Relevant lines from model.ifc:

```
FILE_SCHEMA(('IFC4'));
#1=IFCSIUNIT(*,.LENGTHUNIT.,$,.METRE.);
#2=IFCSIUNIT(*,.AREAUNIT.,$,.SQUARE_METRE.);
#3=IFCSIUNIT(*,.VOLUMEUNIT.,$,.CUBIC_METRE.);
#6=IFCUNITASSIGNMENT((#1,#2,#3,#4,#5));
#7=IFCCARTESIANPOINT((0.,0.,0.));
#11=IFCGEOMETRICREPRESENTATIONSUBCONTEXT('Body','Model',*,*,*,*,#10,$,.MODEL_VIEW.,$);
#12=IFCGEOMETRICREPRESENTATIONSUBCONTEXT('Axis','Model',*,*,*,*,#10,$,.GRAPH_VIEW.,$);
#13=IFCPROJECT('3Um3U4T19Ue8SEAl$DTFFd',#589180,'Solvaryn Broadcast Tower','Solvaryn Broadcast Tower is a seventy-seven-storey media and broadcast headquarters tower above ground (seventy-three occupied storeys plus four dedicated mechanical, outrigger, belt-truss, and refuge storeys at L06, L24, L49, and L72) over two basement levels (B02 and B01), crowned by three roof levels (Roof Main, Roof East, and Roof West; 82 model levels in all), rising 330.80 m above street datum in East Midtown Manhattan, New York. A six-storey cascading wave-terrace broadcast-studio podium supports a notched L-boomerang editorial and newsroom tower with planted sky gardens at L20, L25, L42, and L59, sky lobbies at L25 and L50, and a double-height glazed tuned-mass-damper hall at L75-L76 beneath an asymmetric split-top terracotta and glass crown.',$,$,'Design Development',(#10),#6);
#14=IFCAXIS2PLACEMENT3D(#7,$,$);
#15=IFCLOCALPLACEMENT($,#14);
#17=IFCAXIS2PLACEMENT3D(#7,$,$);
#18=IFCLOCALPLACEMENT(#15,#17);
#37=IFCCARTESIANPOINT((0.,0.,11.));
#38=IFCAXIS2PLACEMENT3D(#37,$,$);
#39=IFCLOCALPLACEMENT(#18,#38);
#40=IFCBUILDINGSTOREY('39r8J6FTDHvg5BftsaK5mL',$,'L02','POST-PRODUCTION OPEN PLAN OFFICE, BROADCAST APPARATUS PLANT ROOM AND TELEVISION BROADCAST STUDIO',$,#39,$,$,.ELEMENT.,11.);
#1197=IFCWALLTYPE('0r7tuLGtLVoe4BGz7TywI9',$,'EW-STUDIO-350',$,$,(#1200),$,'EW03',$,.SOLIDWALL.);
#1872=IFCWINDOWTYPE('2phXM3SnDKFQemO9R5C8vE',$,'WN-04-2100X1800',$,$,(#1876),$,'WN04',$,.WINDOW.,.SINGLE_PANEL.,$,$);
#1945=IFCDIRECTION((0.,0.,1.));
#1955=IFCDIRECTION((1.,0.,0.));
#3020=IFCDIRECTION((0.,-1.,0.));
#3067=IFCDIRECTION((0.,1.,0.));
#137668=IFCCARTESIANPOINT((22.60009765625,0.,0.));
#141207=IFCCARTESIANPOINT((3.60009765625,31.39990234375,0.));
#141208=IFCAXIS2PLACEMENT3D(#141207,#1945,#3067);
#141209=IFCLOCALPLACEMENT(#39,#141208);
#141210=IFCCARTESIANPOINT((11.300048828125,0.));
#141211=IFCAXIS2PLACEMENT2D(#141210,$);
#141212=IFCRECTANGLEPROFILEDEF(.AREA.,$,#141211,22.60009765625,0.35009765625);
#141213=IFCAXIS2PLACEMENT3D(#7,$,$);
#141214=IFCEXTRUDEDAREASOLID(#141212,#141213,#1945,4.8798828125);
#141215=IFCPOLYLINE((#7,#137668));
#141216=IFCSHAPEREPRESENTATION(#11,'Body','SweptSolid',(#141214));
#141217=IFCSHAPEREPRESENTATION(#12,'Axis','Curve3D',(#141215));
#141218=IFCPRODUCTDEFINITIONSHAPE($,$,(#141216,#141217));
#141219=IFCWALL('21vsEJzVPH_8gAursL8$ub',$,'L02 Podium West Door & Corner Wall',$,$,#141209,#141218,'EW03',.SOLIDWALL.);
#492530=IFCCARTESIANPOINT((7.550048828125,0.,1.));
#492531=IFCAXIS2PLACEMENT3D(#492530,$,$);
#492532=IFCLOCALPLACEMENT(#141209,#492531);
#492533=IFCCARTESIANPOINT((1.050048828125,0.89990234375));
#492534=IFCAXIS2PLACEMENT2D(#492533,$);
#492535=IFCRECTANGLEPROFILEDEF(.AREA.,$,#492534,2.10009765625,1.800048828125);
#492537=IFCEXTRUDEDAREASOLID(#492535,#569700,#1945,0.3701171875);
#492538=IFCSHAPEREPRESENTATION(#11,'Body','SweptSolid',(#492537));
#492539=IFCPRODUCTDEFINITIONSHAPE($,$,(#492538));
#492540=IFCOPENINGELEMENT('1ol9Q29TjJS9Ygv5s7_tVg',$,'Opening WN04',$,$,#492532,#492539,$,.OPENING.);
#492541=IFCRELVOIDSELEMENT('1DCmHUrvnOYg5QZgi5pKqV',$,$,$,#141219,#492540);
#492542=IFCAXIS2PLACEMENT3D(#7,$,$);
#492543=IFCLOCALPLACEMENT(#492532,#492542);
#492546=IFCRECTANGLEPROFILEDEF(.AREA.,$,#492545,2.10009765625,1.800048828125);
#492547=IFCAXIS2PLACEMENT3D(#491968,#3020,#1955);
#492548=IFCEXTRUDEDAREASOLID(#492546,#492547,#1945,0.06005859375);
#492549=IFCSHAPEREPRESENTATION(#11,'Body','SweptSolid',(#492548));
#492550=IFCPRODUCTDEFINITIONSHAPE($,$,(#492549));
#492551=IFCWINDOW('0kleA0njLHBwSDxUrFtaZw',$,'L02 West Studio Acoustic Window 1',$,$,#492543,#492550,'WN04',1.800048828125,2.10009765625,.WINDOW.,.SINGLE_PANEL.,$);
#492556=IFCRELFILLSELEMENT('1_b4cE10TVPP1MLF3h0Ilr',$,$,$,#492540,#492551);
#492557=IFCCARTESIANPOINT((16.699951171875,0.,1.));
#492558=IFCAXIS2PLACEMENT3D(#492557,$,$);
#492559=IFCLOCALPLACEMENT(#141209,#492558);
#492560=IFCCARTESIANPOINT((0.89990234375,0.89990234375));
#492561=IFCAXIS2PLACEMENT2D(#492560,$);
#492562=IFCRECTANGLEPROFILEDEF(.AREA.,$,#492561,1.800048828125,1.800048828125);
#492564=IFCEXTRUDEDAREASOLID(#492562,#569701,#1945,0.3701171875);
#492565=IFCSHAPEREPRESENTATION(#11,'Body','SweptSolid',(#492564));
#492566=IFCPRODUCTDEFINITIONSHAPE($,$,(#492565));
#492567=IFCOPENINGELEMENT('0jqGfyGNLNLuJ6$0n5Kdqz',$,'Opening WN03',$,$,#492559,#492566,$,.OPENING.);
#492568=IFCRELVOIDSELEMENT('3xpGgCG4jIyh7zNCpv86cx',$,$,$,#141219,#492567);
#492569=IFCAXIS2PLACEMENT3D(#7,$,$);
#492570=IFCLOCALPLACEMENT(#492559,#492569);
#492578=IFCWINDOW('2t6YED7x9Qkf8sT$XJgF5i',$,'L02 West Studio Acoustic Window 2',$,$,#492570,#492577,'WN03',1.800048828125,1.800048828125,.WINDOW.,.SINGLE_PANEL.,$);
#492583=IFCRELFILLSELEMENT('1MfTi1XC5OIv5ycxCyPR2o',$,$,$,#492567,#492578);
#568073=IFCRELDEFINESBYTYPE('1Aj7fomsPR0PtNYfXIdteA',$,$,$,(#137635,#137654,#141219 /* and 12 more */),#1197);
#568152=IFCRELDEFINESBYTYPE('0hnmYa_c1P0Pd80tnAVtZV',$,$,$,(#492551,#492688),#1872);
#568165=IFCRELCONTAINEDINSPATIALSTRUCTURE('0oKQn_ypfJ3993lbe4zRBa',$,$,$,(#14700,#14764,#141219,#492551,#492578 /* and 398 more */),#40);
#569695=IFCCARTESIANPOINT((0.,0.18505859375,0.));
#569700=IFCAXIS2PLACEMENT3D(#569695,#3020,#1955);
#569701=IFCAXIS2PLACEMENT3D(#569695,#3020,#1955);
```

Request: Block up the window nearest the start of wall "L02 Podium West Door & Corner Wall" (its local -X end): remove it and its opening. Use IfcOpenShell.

```python
import ifcopenshell
import ifcopenshell.api.feature
import ifcopenshell.api.root
import ifcopenshell.geom
import ifcopenshell.util.shape

model = ifcopenshell.open("model.ifc")
settings = ifcopenshell.geom.settings()


def volume(element):
    """Net volume in cubic metres, openings subtracted."""
    shape = ifcopenshell.geom.create_shape(settings, element)
    return ifcopenshell.util.shape.get_volume(shape.geometry)


window = model.by_id(492551)
opening = window.FillsVoids[0].RelatingOpeningElement
wall = opening.VoidsElements[0].RelatingBuildingElement
before = volume(wall)

ifcopenshell.api.root.remove_product(model, product=window)
ifcopenshell.api.feature.remove_feature(model, feature=opening)

after = volume(wall)

print(f"wall volume {before:.3f} -> {after:.3f} m3")

model.write("model-out.ifc")
```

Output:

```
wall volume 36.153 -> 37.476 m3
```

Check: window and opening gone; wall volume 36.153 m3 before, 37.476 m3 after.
